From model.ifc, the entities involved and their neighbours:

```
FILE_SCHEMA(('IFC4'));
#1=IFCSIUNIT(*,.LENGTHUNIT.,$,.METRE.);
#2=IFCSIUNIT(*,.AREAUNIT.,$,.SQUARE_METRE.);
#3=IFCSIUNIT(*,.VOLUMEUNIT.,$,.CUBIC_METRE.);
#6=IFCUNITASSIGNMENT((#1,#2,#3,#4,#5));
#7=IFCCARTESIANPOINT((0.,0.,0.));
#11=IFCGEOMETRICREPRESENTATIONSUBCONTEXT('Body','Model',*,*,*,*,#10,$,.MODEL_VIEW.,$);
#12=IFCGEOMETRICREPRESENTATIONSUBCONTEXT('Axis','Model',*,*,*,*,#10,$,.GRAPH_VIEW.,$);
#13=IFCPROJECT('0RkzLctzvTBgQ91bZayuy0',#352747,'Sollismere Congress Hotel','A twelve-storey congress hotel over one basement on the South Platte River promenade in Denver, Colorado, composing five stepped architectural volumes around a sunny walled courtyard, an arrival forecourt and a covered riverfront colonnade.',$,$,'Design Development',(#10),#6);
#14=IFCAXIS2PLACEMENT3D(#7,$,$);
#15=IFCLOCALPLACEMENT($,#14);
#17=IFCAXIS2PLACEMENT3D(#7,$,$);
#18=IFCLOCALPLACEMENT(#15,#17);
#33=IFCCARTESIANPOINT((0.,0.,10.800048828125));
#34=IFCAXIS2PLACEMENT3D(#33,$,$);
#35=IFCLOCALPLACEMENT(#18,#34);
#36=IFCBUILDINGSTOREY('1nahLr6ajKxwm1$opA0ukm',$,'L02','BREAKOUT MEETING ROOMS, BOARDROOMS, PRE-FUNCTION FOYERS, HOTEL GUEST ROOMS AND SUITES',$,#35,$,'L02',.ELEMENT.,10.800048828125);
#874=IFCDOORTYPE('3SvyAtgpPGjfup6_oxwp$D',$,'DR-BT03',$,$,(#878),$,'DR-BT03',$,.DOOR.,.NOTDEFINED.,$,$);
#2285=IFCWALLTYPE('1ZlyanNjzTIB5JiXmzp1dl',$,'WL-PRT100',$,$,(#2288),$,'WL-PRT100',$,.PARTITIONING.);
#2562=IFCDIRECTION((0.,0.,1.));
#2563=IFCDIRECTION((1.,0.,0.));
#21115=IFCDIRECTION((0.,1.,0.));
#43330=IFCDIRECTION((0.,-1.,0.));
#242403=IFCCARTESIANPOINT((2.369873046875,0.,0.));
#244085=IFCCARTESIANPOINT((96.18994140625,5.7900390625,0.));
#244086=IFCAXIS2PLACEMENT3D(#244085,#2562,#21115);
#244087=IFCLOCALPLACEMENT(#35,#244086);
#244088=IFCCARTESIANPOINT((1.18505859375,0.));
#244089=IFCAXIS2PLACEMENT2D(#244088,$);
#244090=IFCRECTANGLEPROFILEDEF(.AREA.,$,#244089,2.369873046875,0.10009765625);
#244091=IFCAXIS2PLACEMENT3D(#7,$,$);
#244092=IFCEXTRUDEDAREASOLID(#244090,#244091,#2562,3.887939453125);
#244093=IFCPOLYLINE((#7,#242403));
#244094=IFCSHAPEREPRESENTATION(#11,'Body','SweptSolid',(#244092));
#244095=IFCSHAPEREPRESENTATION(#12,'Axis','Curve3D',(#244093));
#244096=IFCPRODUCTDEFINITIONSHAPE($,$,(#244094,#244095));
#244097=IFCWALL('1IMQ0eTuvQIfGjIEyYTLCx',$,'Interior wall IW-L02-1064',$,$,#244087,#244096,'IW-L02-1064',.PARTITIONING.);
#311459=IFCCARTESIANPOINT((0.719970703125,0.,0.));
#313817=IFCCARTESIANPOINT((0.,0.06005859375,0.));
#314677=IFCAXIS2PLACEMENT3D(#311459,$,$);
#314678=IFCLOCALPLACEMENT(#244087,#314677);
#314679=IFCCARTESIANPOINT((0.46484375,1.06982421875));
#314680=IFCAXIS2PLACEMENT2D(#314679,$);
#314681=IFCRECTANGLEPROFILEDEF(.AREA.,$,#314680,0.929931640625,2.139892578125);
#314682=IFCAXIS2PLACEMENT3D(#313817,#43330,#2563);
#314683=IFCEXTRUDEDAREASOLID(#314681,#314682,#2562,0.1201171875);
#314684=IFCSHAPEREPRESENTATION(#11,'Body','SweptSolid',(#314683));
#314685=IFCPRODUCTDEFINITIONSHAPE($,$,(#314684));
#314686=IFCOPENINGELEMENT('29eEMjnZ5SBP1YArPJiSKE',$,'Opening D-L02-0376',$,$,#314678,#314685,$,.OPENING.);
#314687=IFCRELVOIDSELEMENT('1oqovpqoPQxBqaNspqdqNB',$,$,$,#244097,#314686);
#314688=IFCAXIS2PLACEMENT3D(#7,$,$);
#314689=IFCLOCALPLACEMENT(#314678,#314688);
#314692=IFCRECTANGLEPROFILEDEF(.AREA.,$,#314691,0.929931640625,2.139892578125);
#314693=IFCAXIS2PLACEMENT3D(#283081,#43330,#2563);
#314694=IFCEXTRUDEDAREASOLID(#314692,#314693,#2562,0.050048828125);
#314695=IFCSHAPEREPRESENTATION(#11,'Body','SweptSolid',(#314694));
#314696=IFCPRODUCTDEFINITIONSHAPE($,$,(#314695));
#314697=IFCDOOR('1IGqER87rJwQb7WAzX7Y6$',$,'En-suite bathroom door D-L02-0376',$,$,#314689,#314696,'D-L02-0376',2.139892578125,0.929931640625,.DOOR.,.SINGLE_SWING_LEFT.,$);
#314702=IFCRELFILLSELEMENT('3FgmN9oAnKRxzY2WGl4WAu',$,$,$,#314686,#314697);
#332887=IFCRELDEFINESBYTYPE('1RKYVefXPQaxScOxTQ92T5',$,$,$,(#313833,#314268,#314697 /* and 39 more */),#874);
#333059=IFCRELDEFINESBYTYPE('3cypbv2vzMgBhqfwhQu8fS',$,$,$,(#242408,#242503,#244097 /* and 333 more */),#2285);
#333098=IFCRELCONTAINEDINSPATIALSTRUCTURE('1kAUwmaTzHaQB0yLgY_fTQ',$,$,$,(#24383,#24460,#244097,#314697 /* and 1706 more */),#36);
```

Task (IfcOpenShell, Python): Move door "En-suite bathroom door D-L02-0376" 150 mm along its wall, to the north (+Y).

```python
import ifcopenshell
import ifcopenshell.api.geometry
import ifcopenshell.util.placement

model = ifcopenshell.open("model.ifc")

door = model.by_id(314697)
opening = door.FillsVoids[0].RelatingOpeningElement
wall = opening.VoidsElements[0].RelatingBuildingElement

wall_matrix = ifcopenshell.util.placement.get_local_placement(wall.ObjectPlacement)
shift = wall_matrix[:3, 0] * 0.15
before = ifcopenshell.util.placement.get_local_placement(door.ObjectPlacement)[:3, 3].copy()

# The door is placed relative to its opening, so it follows when the opening moves.
matrix = ifcopenshell.util.placement.get_local_placement(opening.ObjectPlacement)
matrix[:3, 3] += shift
ifcopenshell.api.geometry.edit_object_placement(
    model, product=opening, matrix=matrix, is_si=False, should_transform_children=True
)

after = ifcopenshell.util.placement.get_local_placement(door.ObjectPlacement)[:3, 3]
print("door moved by", (after - before).round(3) + 0.0)

model.write("model_edited.ifc")
```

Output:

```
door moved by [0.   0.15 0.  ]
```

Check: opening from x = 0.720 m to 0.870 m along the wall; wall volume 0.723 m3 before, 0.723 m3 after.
